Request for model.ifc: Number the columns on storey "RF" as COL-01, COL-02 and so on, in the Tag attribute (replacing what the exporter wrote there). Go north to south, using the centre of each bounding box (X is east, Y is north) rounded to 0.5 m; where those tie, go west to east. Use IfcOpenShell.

First a look at what the model holds.

```python
import ifcopenshell
import ifcopenshell.util.element
import ifcopenshell.util.placement

model = ifcopenshell.open("model.ifc")
print(model.schema)
storey = next(s for s in model.by_type("IfcBuildingStorey") if s.Name == "RF")
columns = [e for e in ifcopenshell.util.element.get_decomposition(storey) if e.is_a("IfcColumn")]
for e in sorted(columns, key=lambda e: e.id()):
    origin = ifcopenshell.util.placement.get_local_placement(e.ObjectPlacement)[:3, 3]
    print(e.id(), e.Tag, e.Name, origin.round(2) + 0.0, sep=" | ")
```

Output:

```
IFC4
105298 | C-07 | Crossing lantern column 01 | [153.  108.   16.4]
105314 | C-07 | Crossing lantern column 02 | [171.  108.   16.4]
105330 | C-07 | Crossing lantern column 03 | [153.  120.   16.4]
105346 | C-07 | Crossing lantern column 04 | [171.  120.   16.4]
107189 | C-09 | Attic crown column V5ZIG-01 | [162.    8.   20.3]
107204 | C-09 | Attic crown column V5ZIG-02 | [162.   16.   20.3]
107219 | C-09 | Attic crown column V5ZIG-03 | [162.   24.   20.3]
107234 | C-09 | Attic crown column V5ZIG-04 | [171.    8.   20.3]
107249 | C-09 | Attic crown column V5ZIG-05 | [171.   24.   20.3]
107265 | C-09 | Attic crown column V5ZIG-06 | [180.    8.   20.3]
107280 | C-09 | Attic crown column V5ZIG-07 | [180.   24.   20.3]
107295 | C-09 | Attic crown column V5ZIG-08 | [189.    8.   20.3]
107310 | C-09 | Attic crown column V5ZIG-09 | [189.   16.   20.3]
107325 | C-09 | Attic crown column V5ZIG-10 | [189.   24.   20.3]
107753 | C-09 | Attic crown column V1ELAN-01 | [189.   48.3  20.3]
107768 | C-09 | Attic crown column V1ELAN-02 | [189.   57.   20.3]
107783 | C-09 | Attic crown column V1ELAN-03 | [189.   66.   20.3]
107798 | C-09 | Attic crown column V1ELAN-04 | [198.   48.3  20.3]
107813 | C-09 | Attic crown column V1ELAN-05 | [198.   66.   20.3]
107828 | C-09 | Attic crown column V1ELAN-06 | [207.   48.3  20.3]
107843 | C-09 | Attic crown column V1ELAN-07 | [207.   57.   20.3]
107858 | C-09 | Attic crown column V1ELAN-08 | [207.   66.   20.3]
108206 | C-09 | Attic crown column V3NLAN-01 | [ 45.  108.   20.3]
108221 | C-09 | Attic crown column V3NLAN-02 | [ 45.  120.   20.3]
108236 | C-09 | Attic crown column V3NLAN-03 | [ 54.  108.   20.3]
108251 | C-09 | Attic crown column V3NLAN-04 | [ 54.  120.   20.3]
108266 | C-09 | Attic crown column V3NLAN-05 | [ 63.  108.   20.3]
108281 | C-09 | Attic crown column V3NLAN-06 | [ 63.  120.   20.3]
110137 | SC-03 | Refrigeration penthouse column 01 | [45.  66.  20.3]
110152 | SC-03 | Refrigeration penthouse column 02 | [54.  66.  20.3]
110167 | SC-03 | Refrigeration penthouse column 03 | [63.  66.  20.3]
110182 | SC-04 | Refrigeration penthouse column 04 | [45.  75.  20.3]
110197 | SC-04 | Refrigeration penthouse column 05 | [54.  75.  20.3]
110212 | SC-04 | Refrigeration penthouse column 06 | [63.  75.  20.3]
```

```python
import ifcopenshell
import ifcopenshell.geom
import ifcopenshell.util.element
import ifcopenshell.util.shape

model = ifcopenshell.open("model.ifc")
settings = ifcopenshell.geom.settings()
settings.set("use-world-coords", True)


def centre(element):
    shape = ifcopenshell.geom.create_shape(settings, element)
    return ifcopenshell.util.shape.get_bbox_centroid(shape.geometry)


storey = next(s for s in model.by_type("IfcBuildingStorey") if s.Name == "RF")
columns = [e for e in ifcopenshell.util.element.get_decomposition(storey) if e.is_a("IfcColumn")]

# Insertion points can sit at a corner or the storey origin, so sort by the geometry (in metres).
centres = {e: centre(e) for e in columns}
columns.sort(key=lambda e: (-round(centres[e][1] / 0.5), centres[e][0]))

for i, e in enumerate(columns, start=1):
    number = f"COL-{i:02d}"
    e.Tag = number
    print(e.id(), number)

model.write("model_updated.ifc")
```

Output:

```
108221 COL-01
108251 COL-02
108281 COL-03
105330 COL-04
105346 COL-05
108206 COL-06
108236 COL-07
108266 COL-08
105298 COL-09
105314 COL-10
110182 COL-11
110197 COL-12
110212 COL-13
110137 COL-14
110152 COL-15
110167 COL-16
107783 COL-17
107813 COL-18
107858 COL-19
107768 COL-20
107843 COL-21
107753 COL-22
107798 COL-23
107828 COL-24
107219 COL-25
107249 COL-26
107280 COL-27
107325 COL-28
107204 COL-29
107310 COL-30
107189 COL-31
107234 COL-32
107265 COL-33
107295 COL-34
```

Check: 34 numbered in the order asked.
